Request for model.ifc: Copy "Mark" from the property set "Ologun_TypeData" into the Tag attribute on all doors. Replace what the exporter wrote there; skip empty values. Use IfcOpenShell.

First a look at what the model holds.

```python
import ifcopenshell
import ifcopenshell.util.element

model = ifcopenshell.open("model.ifc")
print(model.schema)
doors = model.by_type("IfcDoor")
print(len(doors), "doors")
for e in doors[:8]:
    source = ifcopenshell.util.element.get_pset(e, "Ologun_TypeData", "Mark")
    target = e.Tag
    print(e.id(), repr(source), repr(target), sep=" | ")
```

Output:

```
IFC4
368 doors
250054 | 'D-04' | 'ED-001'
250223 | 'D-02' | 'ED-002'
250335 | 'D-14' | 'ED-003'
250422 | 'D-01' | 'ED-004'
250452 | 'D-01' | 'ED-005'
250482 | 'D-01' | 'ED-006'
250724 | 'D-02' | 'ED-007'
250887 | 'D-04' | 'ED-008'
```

```python
import ifcopenshell
import ifcopenshell.util.element

model = ifcopenshell.open("model.ifc")

count = 0
for e in model.by_type("IfcDoor"):
    value = ifcopenshell.util.element.get_pset(e, "Ologun_TypeData", "Mark")
    current = e.Tag
    if not value or not value.strip() or current == value:
        continue
    e.Tag = value
    count += 1

print(count, "doors updated")

model.write("model_v2.ifc")
```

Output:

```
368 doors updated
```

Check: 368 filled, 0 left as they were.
